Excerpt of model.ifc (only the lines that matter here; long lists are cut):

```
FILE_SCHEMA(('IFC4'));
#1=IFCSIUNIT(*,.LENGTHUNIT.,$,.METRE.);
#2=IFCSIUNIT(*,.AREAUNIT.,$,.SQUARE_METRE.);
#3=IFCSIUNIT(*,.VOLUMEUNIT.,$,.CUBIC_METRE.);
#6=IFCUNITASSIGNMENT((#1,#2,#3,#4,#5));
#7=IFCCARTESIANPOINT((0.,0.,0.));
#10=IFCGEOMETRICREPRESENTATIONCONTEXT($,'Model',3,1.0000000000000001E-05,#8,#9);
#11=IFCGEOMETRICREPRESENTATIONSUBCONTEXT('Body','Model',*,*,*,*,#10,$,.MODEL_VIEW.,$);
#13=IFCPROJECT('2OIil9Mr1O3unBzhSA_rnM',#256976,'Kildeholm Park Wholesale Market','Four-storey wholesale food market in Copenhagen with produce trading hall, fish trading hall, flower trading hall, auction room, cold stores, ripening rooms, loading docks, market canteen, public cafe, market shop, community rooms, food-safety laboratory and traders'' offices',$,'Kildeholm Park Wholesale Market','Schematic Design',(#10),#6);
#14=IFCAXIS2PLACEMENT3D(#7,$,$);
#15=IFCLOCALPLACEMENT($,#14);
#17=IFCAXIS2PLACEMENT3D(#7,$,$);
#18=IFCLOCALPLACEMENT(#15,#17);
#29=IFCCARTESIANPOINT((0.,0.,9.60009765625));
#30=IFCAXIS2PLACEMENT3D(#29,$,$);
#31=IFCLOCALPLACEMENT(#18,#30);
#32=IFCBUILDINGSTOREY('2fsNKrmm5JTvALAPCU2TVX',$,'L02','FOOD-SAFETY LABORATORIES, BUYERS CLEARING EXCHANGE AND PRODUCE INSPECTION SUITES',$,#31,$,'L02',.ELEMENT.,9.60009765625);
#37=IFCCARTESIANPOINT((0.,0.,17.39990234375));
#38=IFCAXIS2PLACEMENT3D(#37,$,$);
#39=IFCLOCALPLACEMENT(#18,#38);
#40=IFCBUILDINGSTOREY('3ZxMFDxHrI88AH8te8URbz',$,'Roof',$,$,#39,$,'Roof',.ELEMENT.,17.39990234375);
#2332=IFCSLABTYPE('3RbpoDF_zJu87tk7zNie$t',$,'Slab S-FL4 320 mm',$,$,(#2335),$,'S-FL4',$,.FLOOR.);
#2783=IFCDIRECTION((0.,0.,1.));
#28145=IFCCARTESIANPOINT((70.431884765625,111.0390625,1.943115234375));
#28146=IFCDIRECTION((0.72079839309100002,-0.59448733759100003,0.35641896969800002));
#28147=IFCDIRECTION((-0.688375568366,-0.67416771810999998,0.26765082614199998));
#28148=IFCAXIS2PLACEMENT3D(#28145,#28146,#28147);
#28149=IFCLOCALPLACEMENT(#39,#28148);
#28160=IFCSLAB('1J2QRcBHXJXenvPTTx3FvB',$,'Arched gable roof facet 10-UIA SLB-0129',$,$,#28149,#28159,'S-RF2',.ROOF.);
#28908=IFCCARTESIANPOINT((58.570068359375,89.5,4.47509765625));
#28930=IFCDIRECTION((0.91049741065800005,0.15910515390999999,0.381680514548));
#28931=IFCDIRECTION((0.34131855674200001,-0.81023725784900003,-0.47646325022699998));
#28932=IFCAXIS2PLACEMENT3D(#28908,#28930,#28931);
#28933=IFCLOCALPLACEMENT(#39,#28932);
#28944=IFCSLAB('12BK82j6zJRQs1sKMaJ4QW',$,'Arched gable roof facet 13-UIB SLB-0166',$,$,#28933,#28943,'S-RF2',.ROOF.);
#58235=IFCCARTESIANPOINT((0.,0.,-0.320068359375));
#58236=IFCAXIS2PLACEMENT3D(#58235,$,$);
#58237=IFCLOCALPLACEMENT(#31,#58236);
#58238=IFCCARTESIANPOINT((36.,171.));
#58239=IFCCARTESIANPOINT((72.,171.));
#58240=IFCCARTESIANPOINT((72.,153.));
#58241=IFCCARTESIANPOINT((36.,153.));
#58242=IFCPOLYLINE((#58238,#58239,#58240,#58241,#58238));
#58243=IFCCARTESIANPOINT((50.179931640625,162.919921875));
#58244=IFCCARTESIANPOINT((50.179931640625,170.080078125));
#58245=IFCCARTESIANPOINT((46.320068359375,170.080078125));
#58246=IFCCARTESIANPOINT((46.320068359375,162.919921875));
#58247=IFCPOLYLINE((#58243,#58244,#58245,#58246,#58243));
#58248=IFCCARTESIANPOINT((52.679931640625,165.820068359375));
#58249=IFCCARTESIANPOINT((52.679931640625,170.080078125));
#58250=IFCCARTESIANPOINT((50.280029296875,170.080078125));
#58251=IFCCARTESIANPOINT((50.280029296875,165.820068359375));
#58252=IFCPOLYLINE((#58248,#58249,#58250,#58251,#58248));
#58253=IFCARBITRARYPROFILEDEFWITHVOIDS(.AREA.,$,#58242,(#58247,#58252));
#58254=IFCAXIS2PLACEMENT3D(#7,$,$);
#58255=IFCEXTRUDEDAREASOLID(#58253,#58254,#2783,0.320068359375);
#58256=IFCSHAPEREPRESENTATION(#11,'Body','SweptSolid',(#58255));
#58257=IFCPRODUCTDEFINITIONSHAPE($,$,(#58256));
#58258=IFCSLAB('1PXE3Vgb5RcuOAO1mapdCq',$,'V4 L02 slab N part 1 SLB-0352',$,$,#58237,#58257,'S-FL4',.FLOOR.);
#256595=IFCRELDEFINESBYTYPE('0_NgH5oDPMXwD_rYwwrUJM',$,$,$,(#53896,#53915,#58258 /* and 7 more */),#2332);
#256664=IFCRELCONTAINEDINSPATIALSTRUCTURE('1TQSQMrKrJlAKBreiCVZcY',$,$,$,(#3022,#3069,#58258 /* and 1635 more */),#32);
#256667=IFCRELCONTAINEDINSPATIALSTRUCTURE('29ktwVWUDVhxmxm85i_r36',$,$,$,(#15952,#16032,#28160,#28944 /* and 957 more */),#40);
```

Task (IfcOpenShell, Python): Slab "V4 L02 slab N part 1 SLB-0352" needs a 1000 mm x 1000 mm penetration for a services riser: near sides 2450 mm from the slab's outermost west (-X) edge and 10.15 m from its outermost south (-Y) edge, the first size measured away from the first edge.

```python
import numpy as np
import ifcopenshell
import ifcopenshell.api.feature
import ifcopenshell.api.geometry
import ifcopenshell.api.root
import ifcopenshell.geom
import ifcopenshell.util.placement
import ifcopenshell.util.representation
import ifcopenshell.util.shape
import ifcopenshell.util.unit

model = ifcopenshell.open("model.ifc")
unit_scale = ifcopenshell.util.unit.calculate_unit_scale(model)
settings = ifcopenshell.geom.settings()


def volume(element):
    """Net volume in cubic metres, openings subtracted."""
    shape = ifcopenshell.geom.create_shape(settings, element)
    return ifcopenshell.util.shape.get_volume(shape.geometry)


slab = model.by_guid("1PXE3Vgb5RcuOAO1mapdCq")
before = volume(slab)

# Extent in the slab's own axes, in metres. The edges named are its -X and -Y sides.
slab_shape = ifcopenshell.geom.create_shape(settings, slab)
vertices = ifcopenshell.util.shape.get_vertices(slab_shape.geometry)
x_min, y_min, bottom = vertices.min(axis=0)
top = vertices[:, 2].max()

opening = ifcopenshell.api.root.create_entity(model, ifc_class="IfcOpeningElement", name="Services riser opening", predefined_type="OPENING")
context = ifcopenshell.util.representation.get_context(model, "Model", "Body", "MODEL_VIEW")
width, depth = 1, 1
outline = [(0.0, 0.0), (width, 0.0), (width, depth), (0.0, depth), (0.0, 0.0)]
# Overshoot both faces by 50 mm so the cut is clean.
shape = ifcopenshell.api.geometry.add_slab_representation(
    model, context=context, depth=top - bottom + 0.1, polyline=outline
)
ifcopenshell.api.geometry.assign_representation(model, product=opening, representation=shape)

matrix = ifcopenshell.util.placement.get_local_placement(slab.ObjectPlacement)
matrix[:, 3] = matrix @ np.append(np.array([x_min + 2.45, y_min + 10.15, bottom - 0.05]) / unit_scale, 1.0)
ifcopenshell.api.geometry.edit_object_placement(model, product=opening, matrix=matrix, is_si=False)
ifcopenshell.api.feature.add_feature(model, feature=opening, element=slab)

after = volume(slab)

print(f"slab volume {before:.3f} -> {after:.3f} m3")

model.write("model_updated.ifc")
```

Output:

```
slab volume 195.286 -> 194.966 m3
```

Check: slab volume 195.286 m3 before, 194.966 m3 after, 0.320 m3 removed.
